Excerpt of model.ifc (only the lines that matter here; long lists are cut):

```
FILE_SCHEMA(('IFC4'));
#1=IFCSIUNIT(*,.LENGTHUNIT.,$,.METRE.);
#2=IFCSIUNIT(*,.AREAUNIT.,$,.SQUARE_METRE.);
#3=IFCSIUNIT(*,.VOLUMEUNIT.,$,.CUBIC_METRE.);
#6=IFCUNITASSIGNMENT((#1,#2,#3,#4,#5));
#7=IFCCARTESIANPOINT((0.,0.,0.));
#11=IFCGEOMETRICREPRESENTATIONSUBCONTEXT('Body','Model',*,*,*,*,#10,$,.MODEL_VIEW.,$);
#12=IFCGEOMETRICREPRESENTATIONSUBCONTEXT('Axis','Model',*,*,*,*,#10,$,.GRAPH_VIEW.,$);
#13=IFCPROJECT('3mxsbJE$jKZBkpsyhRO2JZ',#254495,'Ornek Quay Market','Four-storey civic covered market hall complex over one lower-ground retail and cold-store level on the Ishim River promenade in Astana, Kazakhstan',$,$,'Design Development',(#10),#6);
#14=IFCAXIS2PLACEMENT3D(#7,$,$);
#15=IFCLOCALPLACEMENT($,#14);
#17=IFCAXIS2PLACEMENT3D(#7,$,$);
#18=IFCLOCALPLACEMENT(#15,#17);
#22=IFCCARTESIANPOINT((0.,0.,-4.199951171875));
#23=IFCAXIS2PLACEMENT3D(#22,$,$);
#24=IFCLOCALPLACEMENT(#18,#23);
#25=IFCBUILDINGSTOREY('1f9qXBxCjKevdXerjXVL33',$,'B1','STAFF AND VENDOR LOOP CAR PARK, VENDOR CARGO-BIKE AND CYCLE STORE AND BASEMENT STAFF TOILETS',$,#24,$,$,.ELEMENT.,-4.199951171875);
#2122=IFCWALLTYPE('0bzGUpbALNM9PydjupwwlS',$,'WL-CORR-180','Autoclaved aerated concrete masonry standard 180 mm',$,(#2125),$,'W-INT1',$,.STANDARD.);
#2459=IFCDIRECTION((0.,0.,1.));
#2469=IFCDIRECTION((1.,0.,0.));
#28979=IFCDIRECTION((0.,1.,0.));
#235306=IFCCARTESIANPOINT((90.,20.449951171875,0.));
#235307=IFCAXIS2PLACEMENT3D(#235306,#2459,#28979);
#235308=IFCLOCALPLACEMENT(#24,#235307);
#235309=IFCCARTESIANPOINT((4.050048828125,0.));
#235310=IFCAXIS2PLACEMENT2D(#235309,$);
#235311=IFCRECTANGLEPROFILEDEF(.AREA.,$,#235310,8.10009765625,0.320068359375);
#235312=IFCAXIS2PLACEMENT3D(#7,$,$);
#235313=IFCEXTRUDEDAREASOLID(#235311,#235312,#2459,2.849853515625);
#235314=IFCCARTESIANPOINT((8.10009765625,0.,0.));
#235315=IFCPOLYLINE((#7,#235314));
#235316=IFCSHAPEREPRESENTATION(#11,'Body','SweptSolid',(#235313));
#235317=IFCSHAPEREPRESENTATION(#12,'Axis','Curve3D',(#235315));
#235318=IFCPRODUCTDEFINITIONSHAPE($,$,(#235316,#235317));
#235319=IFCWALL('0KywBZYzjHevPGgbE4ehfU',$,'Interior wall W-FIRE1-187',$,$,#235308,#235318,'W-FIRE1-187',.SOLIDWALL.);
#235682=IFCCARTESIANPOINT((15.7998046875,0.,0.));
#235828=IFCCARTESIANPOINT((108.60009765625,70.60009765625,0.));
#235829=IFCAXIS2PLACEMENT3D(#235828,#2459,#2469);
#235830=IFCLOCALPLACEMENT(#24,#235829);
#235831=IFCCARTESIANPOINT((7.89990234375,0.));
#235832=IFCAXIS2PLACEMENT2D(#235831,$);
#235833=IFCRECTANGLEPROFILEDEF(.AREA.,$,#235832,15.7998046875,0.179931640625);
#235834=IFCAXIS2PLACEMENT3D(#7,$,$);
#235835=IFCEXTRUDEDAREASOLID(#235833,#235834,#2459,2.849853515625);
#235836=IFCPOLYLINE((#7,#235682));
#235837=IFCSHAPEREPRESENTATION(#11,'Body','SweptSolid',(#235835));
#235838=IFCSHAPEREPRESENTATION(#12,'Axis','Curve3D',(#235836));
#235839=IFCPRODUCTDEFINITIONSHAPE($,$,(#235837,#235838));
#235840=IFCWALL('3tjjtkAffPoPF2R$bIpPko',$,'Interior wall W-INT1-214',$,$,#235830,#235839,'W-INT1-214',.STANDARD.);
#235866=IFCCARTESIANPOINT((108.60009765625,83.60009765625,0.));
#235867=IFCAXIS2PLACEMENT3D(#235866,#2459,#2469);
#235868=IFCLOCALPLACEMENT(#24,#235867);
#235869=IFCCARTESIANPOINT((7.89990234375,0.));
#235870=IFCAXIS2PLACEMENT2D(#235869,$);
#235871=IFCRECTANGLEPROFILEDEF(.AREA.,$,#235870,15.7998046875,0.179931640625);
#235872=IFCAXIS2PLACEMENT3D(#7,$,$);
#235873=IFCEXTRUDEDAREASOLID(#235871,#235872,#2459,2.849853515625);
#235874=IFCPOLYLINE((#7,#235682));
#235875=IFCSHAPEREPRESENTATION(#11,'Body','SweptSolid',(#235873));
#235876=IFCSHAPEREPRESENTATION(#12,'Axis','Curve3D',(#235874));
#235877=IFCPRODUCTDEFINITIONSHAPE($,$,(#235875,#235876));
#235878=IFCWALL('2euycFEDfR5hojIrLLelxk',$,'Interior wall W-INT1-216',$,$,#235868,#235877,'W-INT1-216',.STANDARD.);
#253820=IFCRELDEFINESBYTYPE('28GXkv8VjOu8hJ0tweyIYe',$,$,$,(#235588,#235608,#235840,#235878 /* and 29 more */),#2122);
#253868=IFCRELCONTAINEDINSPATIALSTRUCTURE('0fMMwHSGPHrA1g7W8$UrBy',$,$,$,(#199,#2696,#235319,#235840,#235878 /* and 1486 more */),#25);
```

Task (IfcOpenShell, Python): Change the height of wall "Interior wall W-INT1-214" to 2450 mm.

```python
import ifcopenshell
import ifcopenshell.geom
import ifcopenshell.util.representation
import ifcopenshell.util.shape
import ifcopenshell.util.unit

model = ifcopenshell.open("model.ifc")
unit_scale = ifcopenshell.util.unit.calculate_unit_scale(model)
settings = ifcopenshell.geom.settings()


def volume(element):
    """Net volume in cubic metres, openings subtracted."""
    shape = ifcopenshell.geom.create_shape(settings, element)
    return ifcopenshell.util.shape.get_volume(shape.geometry)


wall = model.by_guid("3tjjtkAffPoPF2R$bIpPko")
before = volume(wall)

body = ifcopenshell.util.representation.get_representation(wall, "Model", "Body")
solid = body.Items[0]
old_height = solid.Depth
solid.Depth = 2.45 / unit_scale
after = volume(wall)

print(f"height {old_height:g} -> {solid.Depth:g}, volume {before:.3f} -> {after:.3f} m3")

model.write("model_edited.ifc")
```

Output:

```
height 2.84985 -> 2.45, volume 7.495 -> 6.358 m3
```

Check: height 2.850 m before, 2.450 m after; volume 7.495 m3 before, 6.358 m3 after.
